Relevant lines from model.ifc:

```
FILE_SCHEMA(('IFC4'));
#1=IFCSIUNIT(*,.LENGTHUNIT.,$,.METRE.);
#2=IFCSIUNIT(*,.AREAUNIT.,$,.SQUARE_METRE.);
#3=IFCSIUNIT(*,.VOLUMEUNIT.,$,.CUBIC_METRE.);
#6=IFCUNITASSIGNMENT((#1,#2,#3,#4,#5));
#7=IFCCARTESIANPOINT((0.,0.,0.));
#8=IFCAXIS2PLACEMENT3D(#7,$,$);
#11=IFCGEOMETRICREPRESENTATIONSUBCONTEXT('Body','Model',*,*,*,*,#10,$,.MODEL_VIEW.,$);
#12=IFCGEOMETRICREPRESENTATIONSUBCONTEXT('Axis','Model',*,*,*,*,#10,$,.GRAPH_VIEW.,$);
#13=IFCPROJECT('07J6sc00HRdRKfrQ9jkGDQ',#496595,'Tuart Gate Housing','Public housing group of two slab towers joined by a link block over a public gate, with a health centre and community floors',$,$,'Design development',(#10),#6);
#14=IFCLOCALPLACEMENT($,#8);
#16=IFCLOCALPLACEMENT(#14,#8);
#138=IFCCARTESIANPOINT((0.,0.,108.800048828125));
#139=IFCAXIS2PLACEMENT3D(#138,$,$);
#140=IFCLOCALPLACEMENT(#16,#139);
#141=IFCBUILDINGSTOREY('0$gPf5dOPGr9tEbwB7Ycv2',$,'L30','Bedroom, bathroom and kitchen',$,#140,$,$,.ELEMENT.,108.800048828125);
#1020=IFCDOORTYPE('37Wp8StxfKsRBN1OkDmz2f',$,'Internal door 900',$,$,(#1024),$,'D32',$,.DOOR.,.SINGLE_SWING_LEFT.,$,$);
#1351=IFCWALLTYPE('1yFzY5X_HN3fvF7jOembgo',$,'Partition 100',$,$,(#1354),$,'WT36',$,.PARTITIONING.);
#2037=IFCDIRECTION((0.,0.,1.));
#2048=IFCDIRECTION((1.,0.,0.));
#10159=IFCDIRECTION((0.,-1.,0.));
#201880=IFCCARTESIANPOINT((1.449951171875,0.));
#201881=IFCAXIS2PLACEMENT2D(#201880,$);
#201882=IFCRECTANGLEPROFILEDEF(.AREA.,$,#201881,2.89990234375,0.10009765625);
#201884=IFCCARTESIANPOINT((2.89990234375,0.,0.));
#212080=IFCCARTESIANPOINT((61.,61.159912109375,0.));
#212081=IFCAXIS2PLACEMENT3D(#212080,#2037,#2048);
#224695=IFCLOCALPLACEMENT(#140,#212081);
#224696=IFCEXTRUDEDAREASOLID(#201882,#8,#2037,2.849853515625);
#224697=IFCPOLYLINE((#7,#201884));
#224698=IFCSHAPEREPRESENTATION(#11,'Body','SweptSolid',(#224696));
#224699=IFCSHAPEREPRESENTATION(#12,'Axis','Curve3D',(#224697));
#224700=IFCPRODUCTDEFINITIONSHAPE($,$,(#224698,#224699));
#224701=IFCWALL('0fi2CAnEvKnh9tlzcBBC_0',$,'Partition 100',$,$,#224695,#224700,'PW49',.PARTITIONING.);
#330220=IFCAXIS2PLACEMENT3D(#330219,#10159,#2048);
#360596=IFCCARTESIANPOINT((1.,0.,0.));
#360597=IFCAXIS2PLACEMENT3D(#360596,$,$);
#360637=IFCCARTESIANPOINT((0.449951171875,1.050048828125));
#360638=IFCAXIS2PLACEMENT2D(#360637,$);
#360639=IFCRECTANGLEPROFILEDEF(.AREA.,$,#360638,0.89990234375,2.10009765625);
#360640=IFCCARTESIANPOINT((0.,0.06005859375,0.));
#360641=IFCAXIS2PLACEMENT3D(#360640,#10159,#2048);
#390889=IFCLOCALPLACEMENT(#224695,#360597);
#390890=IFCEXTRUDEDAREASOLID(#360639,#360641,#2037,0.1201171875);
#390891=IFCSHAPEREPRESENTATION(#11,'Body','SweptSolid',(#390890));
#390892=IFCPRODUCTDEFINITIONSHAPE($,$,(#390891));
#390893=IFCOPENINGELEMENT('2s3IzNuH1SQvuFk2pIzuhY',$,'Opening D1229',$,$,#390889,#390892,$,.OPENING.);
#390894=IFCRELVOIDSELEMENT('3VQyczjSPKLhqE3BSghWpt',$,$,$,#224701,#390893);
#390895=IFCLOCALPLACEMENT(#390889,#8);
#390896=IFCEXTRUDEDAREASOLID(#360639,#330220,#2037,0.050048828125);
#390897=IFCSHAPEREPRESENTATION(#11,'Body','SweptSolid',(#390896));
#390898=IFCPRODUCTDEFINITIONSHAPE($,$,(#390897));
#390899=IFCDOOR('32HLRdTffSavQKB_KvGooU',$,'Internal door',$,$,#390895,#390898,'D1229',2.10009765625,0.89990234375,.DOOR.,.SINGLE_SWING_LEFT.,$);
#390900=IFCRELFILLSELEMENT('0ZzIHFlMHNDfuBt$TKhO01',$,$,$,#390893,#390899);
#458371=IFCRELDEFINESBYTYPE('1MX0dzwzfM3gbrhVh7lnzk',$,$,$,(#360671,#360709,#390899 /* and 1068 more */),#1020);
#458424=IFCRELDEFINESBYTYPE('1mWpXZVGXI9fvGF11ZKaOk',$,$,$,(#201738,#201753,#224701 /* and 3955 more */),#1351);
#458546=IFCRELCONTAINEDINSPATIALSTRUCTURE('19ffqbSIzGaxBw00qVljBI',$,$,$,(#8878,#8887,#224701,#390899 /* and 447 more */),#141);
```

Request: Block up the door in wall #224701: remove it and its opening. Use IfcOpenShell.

```python
import ifcopenshell
import ifcopenshell.api.feature
import ifcopenshell.api.root
import ifcopenshell.geom
import ifcopenshell.util.shape

model = ifcopenshell.open("model.ifc")
settings = ifcopenshell.geom.settings()


def volume(element):
    """Net volume in cubic metres, openings subtracted."""
    shape = ifcopenshell.geom.create_shape(settings, element)
    return ifcopenshell.util.shape.get_volume(shape.geometry)


door = model.by_guid("32HLRdTffSavQKB_KvGooU")
opening = door.FillsVoids[0].RelatingOpeningElement
wall = opening.VoidsElements[0].RelatingBuildingElement
before = volume(wall)

ifcopenshell.api.root.remove_product(model, product=door)
ifcopenshell.api.feature.remove_feature(model, feature=opening)

after = volume(wall)

print(f"wall volume {before:.3f} -> {after:.3f} m3")

model.write("model-out.ifc")
```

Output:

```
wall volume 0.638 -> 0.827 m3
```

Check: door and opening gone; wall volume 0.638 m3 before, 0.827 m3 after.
